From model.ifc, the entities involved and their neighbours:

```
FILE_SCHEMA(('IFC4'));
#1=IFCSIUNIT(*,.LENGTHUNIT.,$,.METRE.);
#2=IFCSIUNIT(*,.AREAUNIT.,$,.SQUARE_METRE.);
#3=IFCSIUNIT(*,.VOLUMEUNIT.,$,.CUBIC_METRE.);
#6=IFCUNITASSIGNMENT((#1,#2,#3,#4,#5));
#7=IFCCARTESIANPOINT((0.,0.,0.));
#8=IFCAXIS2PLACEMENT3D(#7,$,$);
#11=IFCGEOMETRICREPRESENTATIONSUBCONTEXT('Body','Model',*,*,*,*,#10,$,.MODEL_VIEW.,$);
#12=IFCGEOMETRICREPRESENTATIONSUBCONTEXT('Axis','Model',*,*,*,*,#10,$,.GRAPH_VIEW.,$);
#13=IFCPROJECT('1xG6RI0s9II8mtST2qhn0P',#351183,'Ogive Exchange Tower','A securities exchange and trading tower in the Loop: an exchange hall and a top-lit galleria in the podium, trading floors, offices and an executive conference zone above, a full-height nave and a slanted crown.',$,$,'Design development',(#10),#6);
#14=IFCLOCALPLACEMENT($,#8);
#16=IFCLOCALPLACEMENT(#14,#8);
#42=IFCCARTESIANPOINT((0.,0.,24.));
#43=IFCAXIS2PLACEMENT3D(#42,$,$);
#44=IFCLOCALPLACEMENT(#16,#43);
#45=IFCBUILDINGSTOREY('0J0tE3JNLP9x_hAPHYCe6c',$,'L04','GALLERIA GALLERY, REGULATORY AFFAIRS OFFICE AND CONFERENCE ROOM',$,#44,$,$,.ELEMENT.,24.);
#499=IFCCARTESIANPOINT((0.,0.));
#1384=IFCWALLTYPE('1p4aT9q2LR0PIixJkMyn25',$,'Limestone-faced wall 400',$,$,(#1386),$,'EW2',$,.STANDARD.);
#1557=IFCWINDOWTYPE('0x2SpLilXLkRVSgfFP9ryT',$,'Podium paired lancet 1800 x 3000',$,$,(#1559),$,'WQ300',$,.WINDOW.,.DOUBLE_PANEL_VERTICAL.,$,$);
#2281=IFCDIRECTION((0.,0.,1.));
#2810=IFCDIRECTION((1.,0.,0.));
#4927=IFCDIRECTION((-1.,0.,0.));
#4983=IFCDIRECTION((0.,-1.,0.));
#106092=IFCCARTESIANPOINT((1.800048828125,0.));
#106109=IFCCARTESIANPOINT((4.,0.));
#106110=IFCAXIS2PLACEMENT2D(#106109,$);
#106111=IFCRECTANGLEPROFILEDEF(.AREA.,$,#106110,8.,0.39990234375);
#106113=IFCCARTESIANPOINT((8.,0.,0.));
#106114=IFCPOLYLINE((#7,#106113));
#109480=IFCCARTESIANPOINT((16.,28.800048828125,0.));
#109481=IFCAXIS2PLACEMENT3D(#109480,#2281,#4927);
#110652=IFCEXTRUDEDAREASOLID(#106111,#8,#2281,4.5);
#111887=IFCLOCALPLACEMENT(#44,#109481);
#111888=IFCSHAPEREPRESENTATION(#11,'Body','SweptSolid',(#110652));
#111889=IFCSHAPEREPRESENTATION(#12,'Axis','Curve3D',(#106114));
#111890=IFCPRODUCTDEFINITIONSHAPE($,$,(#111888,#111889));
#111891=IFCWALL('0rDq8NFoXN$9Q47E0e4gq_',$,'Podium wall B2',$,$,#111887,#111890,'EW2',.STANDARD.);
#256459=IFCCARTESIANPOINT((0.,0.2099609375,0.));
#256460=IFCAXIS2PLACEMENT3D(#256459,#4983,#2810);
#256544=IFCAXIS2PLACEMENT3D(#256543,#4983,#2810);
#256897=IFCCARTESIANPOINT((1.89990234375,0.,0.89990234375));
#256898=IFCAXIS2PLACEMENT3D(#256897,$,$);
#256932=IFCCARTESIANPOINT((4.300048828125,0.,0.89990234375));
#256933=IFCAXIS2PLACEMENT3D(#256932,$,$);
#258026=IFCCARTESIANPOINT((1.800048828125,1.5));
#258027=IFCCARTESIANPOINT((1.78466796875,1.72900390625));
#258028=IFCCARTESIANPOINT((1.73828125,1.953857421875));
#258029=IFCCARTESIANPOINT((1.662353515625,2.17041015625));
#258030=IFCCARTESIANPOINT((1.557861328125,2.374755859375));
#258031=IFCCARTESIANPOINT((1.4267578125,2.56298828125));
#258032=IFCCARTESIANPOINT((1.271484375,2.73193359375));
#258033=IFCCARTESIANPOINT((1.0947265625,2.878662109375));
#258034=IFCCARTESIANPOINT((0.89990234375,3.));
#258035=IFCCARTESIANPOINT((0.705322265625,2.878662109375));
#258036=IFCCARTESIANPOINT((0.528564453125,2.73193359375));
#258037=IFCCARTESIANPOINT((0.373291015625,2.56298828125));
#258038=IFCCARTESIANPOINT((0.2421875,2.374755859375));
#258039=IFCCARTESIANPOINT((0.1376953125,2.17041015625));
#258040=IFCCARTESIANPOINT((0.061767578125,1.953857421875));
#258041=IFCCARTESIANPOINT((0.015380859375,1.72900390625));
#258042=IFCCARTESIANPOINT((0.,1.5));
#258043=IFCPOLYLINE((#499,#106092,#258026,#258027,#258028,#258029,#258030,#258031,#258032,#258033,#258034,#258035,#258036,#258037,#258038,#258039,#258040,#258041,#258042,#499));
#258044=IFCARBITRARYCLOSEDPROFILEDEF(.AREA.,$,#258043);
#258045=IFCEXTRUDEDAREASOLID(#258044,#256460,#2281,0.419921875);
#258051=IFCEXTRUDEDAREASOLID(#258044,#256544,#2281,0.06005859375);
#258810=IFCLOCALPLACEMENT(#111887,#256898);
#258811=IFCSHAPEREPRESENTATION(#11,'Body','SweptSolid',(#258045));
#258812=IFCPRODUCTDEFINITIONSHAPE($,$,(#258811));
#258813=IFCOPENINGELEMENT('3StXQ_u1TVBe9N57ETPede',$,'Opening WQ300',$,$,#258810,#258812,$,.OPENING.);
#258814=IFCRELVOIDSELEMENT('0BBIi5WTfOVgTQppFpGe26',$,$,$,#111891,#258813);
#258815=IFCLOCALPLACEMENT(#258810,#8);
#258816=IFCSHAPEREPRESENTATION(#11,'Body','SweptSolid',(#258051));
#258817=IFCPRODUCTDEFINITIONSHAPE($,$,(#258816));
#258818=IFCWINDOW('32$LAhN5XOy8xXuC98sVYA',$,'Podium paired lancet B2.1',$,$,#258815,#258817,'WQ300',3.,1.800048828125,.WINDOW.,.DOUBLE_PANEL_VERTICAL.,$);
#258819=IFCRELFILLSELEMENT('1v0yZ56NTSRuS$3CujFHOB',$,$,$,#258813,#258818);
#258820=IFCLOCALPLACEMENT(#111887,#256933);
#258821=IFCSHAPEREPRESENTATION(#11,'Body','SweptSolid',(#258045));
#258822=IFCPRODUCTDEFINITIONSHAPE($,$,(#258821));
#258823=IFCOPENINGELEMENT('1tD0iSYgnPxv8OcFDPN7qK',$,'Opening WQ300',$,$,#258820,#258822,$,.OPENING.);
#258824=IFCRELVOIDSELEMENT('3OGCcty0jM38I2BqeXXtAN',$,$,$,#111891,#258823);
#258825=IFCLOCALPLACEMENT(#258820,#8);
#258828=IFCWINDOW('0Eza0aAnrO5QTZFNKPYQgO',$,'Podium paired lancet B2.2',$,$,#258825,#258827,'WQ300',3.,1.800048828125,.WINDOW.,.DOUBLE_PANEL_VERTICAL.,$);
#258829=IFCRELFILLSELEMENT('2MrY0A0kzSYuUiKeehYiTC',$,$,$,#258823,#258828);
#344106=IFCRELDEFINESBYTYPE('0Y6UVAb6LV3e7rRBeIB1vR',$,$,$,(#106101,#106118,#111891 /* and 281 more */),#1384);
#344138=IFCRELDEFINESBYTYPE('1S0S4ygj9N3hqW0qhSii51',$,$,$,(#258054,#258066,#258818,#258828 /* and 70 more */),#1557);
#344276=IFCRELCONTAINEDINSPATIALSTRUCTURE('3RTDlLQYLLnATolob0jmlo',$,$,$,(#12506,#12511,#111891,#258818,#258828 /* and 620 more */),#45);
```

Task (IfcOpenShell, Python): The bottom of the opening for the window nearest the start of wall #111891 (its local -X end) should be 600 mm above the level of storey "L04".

```python
import numpy as np
import ifcopenshell
import ifcopenshell.api.geometry
import ifcopenshell.geom
import ifcopenshell.util.element
import ifcopenshell.util.placement
import ifcopenshell.util.shape
import ifcopenshell.util.unit

model = ifcopenshell.open("model.ifc")
unit_scale = ifcopenshell.util.unit.calculate_unit_scale(model)

window = model.by_guid("32$LAhN5XOy8xXuC98sVYA")
opening = window.FillsVoids[0].RelatingOpeningElement
storey = ifcopenshell.util.element.get_container(window, ifc_class="IfcBuildingStorey")
level = ifcopenshell.util.placement.get_local_placement(storey.ObjectPlacement)[2, 3]

# The opening's origin need not be at the sill, so measure its lowest point.
shape = ifcopenshell.geom.create_shape(ifcopenshell.geom.settings(), opening)
bottom = ifcopenshell.util.shape.get_shape_bottom_elevation(shape, shape.geometry) / unit_scale
dz = level + 0.6 - bottom

shift = np.array([0.0, 0.0, dz])
# The window is placed relative to its opening, so it follows when the opening moves.
matrix = ifcopenshell.util.placement.get_local_placement(opening.ObjectPlacement)
matrix[:3, 3] += shift
ifcopenshell.api.geometry.edit_object_placement(
    model, product=opening, matrix=matrix, is_si=False, should_transform_children=True
)

print(f"moved by {dz * unit_scale:+.3f} m")

model.write("model_rev.ifc")
```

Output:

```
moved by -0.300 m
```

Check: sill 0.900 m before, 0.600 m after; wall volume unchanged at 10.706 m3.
